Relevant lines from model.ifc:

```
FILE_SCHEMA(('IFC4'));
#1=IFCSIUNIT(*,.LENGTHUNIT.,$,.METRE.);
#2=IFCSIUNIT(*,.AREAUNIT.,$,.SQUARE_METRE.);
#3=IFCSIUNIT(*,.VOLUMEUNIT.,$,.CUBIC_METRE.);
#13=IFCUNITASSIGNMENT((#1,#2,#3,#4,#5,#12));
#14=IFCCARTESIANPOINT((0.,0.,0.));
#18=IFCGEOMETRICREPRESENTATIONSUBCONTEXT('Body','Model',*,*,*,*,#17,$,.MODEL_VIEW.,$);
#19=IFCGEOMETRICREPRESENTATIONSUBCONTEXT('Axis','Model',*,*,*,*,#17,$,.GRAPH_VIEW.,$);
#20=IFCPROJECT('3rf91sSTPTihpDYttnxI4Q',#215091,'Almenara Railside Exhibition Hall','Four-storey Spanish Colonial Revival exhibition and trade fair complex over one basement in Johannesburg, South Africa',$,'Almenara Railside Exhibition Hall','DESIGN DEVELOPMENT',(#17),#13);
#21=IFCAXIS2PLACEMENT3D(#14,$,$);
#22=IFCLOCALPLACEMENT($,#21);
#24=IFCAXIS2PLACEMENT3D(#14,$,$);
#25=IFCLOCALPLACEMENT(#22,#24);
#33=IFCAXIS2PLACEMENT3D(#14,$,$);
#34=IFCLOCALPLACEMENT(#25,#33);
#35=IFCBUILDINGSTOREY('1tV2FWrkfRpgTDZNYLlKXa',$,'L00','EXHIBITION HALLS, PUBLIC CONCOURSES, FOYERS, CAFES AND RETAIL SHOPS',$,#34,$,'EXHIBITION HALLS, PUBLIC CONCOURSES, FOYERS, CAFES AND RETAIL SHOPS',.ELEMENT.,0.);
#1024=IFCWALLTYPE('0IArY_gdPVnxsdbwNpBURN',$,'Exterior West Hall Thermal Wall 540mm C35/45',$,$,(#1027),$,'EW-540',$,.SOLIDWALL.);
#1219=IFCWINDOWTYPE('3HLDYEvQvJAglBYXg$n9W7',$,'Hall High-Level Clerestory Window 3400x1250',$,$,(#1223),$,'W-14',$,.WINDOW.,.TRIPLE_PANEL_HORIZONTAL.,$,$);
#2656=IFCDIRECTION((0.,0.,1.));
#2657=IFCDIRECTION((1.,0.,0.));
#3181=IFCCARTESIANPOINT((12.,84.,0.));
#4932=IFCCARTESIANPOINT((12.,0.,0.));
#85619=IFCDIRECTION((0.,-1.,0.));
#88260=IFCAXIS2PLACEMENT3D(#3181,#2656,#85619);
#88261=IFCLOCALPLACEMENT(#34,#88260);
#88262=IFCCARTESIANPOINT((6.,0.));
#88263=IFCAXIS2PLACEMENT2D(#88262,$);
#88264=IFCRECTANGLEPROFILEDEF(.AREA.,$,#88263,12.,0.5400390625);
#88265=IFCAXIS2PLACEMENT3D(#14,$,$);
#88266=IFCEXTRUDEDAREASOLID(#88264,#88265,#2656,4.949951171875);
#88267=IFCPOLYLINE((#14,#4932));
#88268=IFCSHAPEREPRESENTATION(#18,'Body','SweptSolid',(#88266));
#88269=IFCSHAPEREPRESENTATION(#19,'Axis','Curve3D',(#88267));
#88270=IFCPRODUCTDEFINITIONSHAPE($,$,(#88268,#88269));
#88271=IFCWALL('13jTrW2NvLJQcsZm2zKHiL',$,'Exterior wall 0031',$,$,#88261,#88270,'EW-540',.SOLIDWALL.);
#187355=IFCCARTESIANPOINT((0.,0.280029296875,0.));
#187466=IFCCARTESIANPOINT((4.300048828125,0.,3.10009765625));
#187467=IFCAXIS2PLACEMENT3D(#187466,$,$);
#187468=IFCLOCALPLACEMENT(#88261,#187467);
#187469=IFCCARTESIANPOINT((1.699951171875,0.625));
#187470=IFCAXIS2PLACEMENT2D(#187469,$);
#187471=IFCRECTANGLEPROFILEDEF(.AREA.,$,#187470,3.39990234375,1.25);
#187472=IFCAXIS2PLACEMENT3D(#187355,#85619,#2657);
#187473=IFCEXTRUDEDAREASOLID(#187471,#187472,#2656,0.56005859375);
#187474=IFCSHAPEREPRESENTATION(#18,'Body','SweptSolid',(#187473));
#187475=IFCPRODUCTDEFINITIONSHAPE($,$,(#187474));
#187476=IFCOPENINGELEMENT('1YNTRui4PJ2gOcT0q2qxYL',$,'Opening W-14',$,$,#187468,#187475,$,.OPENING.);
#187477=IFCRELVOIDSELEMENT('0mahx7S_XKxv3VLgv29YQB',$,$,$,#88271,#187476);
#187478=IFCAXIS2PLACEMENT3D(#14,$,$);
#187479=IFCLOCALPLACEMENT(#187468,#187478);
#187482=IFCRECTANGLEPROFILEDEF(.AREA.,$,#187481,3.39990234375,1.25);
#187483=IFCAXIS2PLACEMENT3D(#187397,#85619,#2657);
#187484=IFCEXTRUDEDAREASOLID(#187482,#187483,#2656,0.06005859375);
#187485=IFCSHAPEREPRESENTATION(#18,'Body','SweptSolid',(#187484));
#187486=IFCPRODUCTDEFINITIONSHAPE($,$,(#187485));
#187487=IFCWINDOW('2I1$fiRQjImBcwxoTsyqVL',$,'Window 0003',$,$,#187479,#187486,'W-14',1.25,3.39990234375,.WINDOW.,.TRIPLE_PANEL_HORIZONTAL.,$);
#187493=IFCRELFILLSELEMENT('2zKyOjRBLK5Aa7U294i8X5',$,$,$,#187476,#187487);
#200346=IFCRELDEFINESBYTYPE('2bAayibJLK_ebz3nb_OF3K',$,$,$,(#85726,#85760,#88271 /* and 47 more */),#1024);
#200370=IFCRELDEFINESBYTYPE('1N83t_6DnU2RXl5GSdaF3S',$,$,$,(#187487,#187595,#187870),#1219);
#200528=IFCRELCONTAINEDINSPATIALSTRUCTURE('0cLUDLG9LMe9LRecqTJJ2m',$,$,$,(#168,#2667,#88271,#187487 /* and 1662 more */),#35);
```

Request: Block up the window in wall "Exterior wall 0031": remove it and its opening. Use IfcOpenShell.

```python
import ifcopenshell
import ifcopenshell.api.feature
import ifcopenshell.api.root
import ifcopenshell.geom
import ifcopenshell.util.shape

model = ifcopenshell.open("model.ifc")
settings = ifcopenshell.geom.settings()


def volume(element):
    """Net volume in cubic metres, openings subtracted."""
    shape = ifcopenshell.geom.create_shape(settings, element)
    return ifcopenshell.util.shape.get_volume(shape.geometry)


window = model.by_guid("2I1$fiRQjImBcwxoTsyqVL")
opening = window.FillsVoids[0].RelatingOpeningElement
wall = opening.VoidsElements[0].RelatingBuildingElement
before = volume(wall)

ifcopenshell.api.root.remove_product(model, product=window)
ifcopenshell.api.feature.remove_feature(model, feature=opening)

after = volume(wall)

print(f"wall volume {before:.3f} -> {after:.3f} m3")

model.write("model_edited.ifc")
```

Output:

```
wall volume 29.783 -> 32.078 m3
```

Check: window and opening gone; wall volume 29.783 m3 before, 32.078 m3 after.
